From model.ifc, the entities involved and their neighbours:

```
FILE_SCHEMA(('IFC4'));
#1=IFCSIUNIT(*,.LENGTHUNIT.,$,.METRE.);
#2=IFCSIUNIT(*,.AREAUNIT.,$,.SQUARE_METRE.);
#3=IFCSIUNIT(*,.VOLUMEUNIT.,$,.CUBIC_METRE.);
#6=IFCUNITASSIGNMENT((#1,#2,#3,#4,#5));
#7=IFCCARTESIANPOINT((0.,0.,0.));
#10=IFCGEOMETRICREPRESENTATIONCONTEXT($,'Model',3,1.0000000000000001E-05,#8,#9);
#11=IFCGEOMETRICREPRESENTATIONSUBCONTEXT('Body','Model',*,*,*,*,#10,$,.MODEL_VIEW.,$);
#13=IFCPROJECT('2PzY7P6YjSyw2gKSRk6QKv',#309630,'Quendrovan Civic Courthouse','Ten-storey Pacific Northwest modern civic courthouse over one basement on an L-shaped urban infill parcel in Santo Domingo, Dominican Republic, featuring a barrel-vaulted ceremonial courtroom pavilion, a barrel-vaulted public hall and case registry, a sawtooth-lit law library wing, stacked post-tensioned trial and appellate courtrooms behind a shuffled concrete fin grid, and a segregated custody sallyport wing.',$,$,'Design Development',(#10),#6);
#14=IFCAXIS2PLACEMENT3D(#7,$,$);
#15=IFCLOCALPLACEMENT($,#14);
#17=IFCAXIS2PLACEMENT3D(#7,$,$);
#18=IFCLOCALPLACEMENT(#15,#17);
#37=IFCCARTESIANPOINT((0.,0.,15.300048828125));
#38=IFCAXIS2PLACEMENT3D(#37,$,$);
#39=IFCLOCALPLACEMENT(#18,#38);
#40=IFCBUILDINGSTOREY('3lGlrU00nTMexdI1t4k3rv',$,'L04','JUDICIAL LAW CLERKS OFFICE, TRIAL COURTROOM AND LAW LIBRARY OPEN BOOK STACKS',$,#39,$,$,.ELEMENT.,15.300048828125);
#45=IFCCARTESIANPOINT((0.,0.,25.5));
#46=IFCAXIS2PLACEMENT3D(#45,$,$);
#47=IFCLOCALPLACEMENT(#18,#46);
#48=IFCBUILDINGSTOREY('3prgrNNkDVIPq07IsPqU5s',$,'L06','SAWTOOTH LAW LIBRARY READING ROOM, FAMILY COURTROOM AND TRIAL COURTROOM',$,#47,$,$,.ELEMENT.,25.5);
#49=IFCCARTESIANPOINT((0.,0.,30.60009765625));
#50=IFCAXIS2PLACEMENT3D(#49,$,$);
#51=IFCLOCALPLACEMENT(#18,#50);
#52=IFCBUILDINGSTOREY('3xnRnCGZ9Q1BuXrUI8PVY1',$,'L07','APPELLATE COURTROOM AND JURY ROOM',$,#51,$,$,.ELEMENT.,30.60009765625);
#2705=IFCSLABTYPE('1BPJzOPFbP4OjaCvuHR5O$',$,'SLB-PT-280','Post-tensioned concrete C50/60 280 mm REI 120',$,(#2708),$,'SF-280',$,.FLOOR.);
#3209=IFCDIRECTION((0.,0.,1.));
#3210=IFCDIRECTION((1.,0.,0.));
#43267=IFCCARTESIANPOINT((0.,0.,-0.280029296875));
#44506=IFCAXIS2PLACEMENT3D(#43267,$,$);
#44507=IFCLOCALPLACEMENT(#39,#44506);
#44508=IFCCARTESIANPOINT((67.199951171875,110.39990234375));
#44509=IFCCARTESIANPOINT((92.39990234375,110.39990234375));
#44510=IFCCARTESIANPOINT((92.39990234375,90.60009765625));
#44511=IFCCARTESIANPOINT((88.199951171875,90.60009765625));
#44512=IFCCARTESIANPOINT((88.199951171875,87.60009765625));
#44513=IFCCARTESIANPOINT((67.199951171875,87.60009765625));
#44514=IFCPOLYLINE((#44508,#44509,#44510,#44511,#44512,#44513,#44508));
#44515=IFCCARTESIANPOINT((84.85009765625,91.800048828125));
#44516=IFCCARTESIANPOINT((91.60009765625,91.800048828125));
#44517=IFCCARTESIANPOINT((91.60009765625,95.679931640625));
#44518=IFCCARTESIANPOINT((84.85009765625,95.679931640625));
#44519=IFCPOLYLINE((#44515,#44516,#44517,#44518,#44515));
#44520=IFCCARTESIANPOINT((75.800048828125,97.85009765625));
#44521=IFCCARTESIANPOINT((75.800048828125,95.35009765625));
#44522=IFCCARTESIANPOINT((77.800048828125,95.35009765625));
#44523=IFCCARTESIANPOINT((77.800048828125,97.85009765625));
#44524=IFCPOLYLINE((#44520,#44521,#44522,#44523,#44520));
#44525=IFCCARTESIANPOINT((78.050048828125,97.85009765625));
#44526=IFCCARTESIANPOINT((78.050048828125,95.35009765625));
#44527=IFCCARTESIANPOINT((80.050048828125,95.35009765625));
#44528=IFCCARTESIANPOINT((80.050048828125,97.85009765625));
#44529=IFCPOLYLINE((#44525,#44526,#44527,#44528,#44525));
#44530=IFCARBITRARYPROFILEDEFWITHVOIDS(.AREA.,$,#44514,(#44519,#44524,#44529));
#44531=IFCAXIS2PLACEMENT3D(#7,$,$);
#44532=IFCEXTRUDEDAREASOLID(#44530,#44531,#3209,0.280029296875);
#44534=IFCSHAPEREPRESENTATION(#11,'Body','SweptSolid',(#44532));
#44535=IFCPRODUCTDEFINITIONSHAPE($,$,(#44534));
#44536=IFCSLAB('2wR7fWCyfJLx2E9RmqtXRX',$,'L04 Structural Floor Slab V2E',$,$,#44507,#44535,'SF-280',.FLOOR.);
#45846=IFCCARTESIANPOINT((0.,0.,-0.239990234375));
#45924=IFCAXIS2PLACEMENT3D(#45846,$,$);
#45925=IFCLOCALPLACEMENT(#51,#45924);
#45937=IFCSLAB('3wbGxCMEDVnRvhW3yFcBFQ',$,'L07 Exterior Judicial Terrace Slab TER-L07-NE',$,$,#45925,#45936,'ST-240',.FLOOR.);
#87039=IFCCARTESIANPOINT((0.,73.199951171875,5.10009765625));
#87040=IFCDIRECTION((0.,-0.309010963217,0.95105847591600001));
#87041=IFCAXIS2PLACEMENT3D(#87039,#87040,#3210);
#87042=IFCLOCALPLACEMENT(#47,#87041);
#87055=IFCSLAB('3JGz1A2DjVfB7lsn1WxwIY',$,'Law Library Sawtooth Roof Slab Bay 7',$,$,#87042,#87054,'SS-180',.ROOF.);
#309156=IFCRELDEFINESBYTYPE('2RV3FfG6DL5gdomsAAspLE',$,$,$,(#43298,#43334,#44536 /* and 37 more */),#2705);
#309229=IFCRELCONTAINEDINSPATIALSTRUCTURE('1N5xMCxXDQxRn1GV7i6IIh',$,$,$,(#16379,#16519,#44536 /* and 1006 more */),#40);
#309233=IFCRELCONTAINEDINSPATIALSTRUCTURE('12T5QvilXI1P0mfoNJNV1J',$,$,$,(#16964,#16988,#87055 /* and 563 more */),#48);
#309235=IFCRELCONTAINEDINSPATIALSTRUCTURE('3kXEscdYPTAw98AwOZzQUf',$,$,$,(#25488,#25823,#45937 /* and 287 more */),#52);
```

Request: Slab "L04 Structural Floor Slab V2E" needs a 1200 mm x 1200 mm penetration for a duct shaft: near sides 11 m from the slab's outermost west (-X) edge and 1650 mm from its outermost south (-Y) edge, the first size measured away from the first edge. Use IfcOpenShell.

```python
import numpy as np
import ifcopenshell
import ifcopenshell.api.feature
import ifcopenshell.api.geometry
import ifcopenshell.api.root
import ifcopenshell.geom
import ifcopenshell.util.placement
import ifcopenshell.util.representation
import ifcopenshell.util.shape
import ifcopenshell.util.unit

model = ifcopenshell.open("model.ifc")
unit_scale = ifcopenshell.util.unit.calculate_unit_scale(model)
settings = ifcopenshell.geom.settings()


def volume(element):
    """Net volume in cubic metres, openings subtracted."""
    shape = ifcopenshell.geom.create_shape(settings, element)
    return ifcopenshell.util.shape.get_volume(shape.geometry)


slab = model.by_guid("2wR7fWCyfJLx2E9RmqtXRX")
before = volume(slab)

# Extent in the slab's own axes, in metres. The edges named are its -X and -Y sides.
slab_shape = ifcopenshell.geom.create_shape(settings, slab)
vertices = ifcopenshell.util.shape.get_vertices(slab_shape.geometry)
x_min, y_min, bottom = vertices.min(axis=0)
top = vertices[:, 2].max()

opening = ifcopenshell.api.root.create_entity(model, ifc_class="IfcOpeningElement", name="Duct shaft opening", predefined_type="OPENING")
context = ifcopenshell.util.representation.get_context(model, "Model", "Body", "MODEL_VIEW")
width, depth = 1.2, 1.2
outline = [(0.0, 0.0), (width, 0.0), (width, depth), (0.0, depth), (0.0, 0.0)]
# Overshoot both faces by 50 mm so the cut is clean.
shape = ifcopenshell.api.geometry.add_slab_representation(
    model, context=context, depth=top - bottom + 0.1, polyline=outline
)
ifcopenshell.api.geometry.assign_representation(model, product=opening, representation=shape)

matrix = ifcopenshell.util.placement.get_local_placement(slab.ObjectPlacement)
matrix[:, 3] = matrix @ np.append(np.array([x_min + 11, y_min + 1.65, bottom - 0.05]) / unit_scale, 1.0)
ifcopenshell.api.geometry.edit_object_placement(model, product=opening, matrix=matrix, is_si=False)
ifcopenshell.api.feature.add_feature(model, feature=opening, element=slab)

after = volume(slab)

print(f"slab volume {before:.3f} -> {after:.3f} m3")

model.write("model_v2.ifc")
```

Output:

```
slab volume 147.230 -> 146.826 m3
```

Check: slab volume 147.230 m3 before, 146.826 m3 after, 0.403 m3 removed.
